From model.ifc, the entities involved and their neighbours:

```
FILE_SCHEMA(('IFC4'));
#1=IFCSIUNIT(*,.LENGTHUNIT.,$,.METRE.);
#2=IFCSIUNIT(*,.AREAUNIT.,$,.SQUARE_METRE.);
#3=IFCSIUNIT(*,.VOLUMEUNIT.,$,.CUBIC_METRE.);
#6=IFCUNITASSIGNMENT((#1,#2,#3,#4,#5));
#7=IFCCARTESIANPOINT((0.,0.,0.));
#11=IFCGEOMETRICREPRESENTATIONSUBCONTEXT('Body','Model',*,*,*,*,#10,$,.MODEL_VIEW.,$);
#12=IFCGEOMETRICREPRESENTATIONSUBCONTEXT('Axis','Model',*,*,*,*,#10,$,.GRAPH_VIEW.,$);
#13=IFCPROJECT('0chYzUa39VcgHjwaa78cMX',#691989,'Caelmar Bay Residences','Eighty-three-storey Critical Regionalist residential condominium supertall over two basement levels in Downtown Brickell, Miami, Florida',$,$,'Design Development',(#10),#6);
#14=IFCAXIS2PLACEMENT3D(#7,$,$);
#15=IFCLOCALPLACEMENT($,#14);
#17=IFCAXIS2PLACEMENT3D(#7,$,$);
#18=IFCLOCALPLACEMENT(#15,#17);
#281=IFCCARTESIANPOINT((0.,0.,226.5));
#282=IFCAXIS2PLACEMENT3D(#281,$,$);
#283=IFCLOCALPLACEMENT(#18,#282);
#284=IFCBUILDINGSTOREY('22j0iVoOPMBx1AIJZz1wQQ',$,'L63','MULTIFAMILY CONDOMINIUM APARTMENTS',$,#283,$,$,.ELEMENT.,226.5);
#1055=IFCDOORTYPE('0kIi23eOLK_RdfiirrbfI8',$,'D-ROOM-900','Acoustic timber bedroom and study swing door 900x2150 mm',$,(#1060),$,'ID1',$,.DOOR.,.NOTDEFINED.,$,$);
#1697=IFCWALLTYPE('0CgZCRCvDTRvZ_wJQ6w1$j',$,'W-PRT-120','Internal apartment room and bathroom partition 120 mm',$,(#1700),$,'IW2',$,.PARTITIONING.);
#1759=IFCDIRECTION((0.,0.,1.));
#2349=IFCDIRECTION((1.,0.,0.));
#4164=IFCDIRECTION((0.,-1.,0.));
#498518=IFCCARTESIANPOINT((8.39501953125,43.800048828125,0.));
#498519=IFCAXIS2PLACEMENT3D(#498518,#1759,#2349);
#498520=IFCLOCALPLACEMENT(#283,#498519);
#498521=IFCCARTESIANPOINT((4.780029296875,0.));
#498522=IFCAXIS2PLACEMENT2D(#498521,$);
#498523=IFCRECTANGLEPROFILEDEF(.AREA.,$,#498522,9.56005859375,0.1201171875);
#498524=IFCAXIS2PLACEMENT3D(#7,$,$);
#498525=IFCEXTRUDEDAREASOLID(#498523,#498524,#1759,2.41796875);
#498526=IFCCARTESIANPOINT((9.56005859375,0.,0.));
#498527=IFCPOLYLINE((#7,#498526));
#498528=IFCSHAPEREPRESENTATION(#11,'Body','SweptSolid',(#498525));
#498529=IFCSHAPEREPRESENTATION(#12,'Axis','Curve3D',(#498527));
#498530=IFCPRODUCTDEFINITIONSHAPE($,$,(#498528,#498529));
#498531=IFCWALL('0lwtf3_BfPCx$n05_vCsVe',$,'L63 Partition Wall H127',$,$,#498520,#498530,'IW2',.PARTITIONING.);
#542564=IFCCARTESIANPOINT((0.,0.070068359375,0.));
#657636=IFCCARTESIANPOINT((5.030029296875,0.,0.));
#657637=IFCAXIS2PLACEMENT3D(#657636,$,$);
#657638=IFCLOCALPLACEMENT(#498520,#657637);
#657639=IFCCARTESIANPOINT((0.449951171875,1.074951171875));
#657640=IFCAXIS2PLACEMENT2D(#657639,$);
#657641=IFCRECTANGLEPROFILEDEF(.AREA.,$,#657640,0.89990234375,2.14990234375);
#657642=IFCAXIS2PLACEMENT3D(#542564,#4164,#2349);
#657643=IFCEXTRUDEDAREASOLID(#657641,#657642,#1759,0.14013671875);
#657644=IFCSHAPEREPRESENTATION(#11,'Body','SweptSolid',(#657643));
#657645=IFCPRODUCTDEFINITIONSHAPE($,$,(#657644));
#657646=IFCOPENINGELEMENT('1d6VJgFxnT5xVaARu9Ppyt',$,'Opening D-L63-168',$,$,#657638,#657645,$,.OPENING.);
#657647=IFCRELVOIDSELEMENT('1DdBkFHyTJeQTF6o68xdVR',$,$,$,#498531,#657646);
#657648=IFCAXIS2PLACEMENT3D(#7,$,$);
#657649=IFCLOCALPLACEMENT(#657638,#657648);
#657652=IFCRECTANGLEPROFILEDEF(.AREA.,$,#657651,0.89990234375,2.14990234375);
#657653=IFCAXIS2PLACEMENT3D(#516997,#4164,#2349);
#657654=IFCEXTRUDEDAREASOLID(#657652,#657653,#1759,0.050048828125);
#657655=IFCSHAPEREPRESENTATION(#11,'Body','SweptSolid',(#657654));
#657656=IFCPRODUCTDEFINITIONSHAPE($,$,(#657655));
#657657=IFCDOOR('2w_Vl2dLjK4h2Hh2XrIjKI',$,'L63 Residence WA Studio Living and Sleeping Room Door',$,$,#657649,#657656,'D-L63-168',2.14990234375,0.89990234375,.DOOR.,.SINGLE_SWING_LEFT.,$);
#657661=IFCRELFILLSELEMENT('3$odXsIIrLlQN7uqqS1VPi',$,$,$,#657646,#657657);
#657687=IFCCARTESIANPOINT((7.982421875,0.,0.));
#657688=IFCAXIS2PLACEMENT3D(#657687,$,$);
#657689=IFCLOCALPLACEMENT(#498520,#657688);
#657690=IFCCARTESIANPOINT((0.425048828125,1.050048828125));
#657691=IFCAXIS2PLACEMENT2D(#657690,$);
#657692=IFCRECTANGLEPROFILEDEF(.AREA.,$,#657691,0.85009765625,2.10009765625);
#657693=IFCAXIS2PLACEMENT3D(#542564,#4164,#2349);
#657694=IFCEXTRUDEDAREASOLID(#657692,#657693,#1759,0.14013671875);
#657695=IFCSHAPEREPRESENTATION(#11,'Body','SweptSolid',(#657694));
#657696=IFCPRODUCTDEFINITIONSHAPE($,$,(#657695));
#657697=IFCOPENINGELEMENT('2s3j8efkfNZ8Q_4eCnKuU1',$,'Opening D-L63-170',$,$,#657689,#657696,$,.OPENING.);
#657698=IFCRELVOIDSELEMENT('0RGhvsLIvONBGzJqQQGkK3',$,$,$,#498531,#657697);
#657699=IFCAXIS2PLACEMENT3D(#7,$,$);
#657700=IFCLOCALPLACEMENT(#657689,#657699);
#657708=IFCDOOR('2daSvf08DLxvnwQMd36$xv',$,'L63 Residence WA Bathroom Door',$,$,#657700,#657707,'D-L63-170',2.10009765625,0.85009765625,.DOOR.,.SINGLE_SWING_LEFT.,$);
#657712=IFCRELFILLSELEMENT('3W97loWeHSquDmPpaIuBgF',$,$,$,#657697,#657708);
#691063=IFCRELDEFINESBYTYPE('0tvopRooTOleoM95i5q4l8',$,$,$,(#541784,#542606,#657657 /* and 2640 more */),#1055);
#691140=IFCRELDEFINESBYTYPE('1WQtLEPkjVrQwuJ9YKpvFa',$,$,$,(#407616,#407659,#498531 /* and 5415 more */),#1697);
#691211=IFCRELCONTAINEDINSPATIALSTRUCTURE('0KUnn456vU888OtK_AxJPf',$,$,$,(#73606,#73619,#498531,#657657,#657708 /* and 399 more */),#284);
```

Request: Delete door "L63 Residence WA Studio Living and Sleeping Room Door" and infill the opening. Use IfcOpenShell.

```python
import ifcopenshell
import ifcopenshell.api.feature
import ifcopenshell.api.root
import ifcopenshell.geom
import ifcopenshell.util.shape

model = ifcopenshell.open("model.ifc")
settings = ifcopenshell.geom.settings()


def volume(element):
    """Net volume in cubic metres, openings subtracted."""
    shape = ifcopenshell.geom.create_shape(settings, element)
    return ifcopenshell.util.shape.get_volume(shape.geometry)


door = model.by_guid("2w_Vl2dLjK4h2Hh2XrIjKI")
opening = door.FillsVoids[0].RelatingOpeningElement
wall = opening.VoidsElements[0].RelatingBuildingElement
before = volume(wall)

ifcopenshell.api.root.remove_product(model, product=door)
ifcopenshell.api.feature.remove_feature(model, feature=opening)

after = volume(wall)

print(f"wall volume {before:.3f} -> {after:.3f} m3")

model.write("model_updated.ifc")
```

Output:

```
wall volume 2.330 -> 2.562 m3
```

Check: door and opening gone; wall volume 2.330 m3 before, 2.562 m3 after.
